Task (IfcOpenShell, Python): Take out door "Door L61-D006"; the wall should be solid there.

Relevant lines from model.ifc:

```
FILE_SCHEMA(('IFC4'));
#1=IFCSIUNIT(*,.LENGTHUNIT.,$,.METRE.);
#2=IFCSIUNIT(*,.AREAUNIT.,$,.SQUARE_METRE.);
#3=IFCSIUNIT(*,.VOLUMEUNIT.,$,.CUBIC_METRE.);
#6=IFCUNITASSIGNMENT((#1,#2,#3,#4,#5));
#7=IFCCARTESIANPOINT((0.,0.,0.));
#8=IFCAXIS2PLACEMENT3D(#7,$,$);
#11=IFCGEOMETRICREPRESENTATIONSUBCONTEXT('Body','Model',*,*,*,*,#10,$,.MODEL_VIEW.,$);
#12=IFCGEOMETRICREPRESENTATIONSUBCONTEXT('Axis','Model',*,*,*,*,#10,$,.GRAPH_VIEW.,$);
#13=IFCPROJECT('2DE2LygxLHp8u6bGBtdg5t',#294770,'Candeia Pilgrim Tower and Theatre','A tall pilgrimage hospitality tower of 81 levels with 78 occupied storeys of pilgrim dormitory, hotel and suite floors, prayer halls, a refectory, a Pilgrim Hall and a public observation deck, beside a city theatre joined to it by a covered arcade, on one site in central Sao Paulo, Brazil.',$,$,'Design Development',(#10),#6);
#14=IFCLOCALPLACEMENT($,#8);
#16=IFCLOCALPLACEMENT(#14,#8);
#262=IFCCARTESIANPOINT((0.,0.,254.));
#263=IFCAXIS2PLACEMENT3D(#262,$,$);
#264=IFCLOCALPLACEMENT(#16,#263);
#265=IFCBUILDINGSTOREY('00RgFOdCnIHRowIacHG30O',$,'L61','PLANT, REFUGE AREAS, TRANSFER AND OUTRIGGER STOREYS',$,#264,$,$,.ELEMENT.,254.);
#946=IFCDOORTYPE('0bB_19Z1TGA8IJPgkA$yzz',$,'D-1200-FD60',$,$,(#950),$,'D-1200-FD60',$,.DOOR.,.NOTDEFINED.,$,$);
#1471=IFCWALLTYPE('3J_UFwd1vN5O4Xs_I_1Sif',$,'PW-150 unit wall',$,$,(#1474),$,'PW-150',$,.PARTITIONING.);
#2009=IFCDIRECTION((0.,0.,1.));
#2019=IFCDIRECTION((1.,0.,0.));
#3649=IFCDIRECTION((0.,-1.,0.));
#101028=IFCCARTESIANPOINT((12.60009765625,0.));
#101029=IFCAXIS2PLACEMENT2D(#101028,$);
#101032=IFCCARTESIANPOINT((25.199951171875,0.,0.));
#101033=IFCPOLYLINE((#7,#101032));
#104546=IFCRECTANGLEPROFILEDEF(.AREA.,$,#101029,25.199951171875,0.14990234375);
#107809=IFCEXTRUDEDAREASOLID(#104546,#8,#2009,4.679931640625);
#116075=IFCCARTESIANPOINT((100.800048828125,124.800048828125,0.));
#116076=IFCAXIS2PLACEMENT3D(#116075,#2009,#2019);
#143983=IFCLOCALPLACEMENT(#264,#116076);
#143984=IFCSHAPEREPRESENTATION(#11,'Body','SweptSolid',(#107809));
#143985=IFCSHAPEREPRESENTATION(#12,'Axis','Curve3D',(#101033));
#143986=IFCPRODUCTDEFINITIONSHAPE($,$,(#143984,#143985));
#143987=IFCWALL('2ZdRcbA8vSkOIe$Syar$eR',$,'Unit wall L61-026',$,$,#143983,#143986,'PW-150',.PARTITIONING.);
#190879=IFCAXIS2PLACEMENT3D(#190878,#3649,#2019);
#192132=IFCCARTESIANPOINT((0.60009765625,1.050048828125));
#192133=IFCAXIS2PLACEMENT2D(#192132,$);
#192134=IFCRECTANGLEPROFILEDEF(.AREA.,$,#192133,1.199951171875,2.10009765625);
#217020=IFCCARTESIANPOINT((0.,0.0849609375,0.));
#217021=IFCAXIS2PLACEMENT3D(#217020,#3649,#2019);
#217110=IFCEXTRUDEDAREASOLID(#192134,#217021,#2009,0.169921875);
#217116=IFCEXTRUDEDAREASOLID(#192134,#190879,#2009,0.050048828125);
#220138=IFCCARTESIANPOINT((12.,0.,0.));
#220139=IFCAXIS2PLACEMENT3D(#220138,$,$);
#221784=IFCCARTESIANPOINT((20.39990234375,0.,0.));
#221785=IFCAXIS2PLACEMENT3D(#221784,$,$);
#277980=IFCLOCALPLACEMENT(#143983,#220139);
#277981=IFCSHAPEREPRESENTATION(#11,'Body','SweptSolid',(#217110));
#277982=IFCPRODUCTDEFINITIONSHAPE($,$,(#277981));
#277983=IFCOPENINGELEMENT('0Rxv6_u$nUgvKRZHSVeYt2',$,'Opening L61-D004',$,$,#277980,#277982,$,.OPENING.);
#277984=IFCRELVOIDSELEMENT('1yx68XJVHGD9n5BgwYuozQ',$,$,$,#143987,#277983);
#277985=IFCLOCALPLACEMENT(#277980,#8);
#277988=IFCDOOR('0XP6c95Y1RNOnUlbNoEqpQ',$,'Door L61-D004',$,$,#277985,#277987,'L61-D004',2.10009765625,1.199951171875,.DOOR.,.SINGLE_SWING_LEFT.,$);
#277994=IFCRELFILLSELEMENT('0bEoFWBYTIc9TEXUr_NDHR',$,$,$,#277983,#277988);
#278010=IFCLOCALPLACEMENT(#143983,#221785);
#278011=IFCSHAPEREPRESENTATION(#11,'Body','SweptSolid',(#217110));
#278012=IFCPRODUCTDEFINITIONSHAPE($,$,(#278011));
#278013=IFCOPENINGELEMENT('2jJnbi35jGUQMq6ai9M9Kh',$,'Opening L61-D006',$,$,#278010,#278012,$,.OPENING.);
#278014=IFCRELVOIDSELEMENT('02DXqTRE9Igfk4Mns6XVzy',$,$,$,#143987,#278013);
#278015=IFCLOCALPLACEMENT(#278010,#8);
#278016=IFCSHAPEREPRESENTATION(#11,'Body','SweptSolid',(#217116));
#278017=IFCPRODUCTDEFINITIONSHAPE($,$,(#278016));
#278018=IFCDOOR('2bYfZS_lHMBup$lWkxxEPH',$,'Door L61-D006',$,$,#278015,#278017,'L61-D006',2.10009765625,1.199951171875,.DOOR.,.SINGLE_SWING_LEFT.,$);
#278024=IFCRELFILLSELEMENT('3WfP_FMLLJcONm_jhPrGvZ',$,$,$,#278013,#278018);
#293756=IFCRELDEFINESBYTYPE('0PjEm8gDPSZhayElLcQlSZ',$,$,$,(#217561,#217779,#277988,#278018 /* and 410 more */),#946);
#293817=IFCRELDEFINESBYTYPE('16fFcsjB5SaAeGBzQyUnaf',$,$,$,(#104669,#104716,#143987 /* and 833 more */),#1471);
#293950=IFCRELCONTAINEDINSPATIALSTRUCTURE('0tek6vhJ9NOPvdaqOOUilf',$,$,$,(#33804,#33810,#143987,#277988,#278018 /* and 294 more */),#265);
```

```python
import ifcopenshell
import ifcopenshell.api.feature
import ifcopenshell.api.root
import ifcopenshell.geom
import ifcopenshell.util.shape

model = ifcopenshell.open("model.ifc")
settings = ifcopenshell.geom.settings()


def volume(element):
    """Net volume in cubic metres, openings subtracted."""
    shape = ifcopenshell.geom.create_shape(settings, element)
    return ifcopenshell.util.shape.get_volume(shape.geometry)


door = model.by_id(278018)
opening = door.FillsVoids[0].RelatingOpeningElement
wall = opening.VoidsElements[0].RelatingBuildingElement
before = volume(wall)

ifcopenshell.api.root.remove_product(model, product=door)
ifcopenshell.api.feature.remove_feature(model, feature=opening)

after = volume(wall)

print(f"wall volume {before:.3f} -> {after:.3f} m3")

model.write("model_edited.ifc")
```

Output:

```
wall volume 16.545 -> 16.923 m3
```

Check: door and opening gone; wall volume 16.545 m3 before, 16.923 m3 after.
